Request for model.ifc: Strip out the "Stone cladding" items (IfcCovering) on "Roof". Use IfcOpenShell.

First a look at what the model holds.

```python
import ifcopenshell
import ifcopenshell.util.element

model = ifcopenshell.open("model.ifc")
print(model.schema)
storey = next(s for s in model.by_type("IfcBuildingStorey") if s.Name == "Roof")
coverings = [e for e in ifcopenshell.util.element.get_decomposition(storey) if e.is_a("IfcCovering")]
seen = {}
for e in coverings:
    element_type = ifcopenshell.util.element.get_type(e)
    name = element_type.Name if element_type not in (None, e) else None
    seen[name] = seen.get(name, 0) + 1
for name, count in sorted(seen.items(), key=str):
    print(count, "x", name)
```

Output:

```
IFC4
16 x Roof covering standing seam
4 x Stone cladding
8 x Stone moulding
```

```python
import ifcopenshell
import ifcopenshell.api.root
import ifcopenshell.util.element

model = ifcopenshell.open("model.ifc")

storey = next(s for s in model.by_type("IfcBuildingStorey") if s.Name == "Roof")
coverings = [e for e in ifcopenshell.util.element.get_decomposition(storey) if e.is_a("IfcCovering")]
targets = [e for e in coverings if (t := ifcopenshell.util.element.get_type(e)) not in (None, e) and t.Name == "Stone cladding"]

for e in targets:
    ifcopenshell.api.root.remove_product(model, product=e)
print(len(targets), "removed")

model.write("model_updated.ifc")
```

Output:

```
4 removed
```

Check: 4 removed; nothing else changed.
